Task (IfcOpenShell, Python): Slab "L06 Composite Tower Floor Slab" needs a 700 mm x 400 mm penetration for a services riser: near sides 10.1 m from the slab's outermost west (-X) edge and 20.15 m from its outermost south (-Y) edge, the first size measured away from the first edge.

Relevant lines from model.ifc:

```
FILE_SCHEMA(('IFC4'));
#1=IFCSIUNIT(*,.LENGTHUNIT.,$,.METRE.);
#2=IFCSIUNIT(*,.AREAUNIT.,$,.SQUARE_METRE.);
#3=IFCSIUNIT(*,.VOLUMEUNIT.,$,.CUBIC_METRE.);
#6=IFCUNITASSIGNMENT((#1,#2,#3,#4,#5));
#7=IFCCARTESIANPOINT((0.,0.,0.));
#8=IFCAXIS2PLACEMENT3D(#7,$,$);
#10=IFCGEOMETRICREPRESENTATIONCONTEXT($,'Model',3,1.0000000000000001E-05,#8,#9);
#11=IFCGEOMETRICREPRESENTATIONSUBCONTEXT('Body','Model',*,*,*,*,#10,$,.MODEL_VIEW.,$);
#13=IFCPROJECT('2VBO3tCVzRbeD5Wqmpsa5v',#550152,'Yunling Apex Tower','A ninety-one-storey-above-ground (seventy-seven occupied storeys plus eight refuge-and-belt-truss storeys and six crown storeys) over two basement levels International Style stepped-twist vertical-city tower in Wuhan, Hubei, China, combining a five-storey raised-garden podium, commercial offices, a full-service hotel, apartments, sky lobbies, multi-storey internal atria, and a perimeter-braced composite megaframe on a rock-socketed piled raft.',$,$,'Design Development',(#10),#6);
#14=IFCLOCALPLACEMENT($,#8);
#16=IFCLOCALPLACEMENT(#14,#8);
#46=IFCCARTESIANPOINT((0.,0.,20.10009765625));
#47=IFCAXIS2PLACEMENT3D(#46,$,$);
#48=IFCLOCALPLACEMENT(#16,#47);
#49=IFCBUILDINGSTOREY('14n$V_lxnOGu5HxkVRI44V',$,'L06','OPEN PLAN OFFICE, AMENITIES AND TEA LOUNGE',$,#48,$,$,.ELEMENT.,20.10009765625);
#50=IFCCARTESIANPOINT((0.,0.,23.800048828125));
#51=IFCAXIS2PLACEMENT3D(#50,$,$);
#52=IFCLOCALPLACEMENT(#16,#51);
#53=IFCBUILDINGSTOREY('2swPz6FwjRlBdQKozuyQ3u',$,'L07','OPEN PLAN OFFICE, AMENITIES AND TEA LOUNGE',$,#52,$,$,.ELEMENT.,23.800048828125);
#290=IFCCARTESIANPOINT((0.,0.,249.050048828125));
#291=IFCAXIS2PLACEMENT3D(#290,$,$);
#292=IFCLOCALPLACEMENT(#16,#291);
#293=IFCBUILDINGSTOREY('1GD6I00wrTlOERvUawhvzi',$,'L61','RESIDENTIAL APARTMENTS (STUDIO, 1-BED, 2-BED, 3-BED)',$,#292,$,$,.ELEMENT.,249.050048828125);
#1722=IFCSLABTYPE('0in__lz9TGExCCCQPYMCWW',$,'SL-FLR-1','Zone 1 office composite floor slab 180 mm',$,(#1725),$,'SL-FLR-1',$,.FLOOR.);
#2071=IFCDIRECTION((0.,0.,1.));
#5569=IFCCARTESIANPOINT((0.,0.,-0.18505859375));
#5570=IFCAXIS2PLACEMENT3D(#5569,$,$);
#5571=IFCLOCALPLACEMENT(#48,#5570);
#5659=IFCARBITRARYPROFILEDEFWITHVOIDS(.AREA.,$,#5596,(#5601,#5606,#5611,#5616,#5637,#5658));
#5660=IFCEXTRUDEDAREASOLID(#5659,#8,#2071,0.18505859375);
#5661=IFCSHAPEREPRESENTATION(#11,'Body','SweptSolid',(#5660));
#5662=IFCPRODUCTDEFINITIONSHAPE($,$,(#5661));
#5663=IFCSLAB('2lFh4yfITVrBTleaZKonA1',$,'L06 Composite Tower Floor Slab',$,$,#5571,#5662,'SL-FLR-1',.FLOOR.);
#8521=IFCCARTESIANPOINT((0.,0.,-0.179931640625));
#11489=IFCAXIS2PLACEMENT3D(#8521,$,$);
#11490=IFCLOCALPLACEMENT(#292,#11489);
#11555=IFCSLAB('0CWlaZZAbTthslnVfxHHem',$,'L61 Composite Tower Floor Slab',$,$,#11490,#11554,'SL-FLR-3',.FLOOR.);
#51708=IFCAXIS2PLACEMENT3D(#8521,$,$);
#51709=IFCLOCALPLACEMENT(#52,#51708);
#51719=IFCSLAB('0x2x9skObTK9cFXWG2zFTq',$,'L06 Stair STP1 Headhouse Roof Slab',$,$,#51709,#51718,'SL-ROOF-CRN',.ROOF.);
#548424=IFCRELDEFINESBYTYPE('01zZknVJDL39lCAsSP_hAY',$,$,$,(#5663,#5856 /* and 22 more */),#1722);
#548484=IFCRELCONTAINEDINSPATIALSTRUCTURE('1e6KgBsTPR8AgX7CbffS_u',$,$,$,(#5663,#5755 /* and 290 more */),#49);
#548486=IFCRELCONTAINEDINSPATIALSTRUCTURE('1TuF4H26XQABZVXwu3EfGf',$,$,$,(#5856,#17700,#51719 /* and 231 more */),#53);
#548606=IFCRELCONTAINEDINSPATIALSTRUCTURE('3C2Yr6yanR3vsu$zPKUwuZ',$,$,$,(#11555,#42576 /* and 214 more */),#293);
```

```python
import numpy as np
import ifcopenshell
import ifcopenshell.api.feature
import ifcopenshell.api.geometry
import ifcopenshell.api.root
import ifcopenshell.geom
import ifcopenshell.util.placement
import ifcopenshell.util.representation
import ifcopenshell.util.shape
import ifcopenshell.util.unit

model = ifcopenshell.open("model.ifc")
unit_scale = ifcopenshell.util.unit.calculate_unit_scale(model)
settings = ifcopenshell.geom.settings()


def volume(element):
    """Net volume in cubic metres, openings subtracted."""
    shape = ifcopenshell.geom.create_shape(settings, element)
    return ifcopenshell.util.shape.get_volume(shape.geometry)


slab = model.by_id(5663)
before = volume(slab)

# Extent in the slab's own axes, in metres. The edges named are its -X and -Y sides.
slab_shape = ifcopenshell.geom.create_shape(settings, slab)
vertices = ifcopenshell.util.shape.get_vertices(slab_shape.geometry)
x_min, y_min, bottom = vertices.min(axis=0)
top = vertices[:, 2].max()

opening = ifcopenshell.api.root.create_entity(model, ifc_class="IfcOpeningElement", name="Services riser opening", predefined_type="OPENING")
context = ifcopenshell.util.representation.get_context(model, "Model", "Body", "MODEL_VIEW")
width, depth = 0.7, 0.4
outline = [(0.0, 0.0), (width, 0.0), (width, depth), (0.0, depth), (0.0, 0.0)]
# Overshoot both faces by 50 mm so the cut is clean.
shape = ifcopenshell.api.geometry.add_slab_representation(
    model, context=context, depth=top - bottom + 0.1, polyline=outline
)
ifcopenshell.api.geometry.assign_representation(model, product=opening, representation=shape)

matrix = ifcopenshell.util.placement.get_local_placement(slab.ObjectPlacement)
matrix[:, 3] = matrix @ np.append(np.array([x_min + 10.1, y_min + 20.15, bottom - 0.05]) / unit_scale, 1.0)
ifcopenshell.api.geometry.edit_object_placement(model, product=opening, matrix=matrix, is_si=False)
ifcopenshell.api.feature.add_feature(model, feature=opening, element=slab)

after = volume(slab)

print(f"slab volume {before:.3f} -> {after:.3f} m3")

model.write("model_v2.ifc")
```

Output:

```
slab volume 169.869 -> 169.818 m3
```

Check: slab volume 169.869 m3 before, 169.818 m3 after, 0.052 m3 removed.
